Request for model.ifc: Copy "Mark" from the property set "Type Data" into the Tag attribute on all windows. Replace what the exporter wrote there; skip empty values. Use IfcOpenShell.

First a look at what the model holds.

```python
import ifcopenshell
import ifcopenshell.util.element

model = ifcopenshell.open("model.ifc")
print(model.schema)
windows = model.by_type("IfcWindow")
print(len(windows), "windows")
for e in windows[:8]:
    source = ifcopenshell.util.element.get_pset(e, "Type Data", "Mark")
    target = e.Tag
    print(e.id(), repr(source), repr(target), sep=" | ")
```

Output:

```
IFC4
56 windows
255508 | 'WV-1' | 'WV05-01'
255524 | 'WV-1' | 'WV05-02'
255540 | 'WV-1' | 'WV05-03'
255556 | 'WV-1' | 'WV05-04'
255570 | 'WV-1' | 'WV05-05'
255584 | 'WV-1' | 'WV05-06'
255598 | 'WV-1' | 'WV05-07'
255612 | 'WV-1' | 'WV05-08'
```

```python
import ifcopenshell
import ifcopenshell.util.element

model = ifcopenshell.open("model.ifc")

count = 0
for e in model.by_type("IfcWindow"):
    value = ifcopenshell.util.element.get_pset(e, "Type Data", "Mark")
    current = e.Tag
    if not value or not value.strip() or current == value:
        continue
    e.Tag = value
    count += 1

print(count, "windows updated")

model.write("model_edited.ifc")
```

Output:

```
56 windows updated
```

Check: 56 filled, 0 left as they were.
